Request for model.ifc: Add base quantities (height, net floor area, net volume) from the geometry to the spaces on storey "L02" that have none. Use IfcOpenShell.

First a look at what the model holds.

```python
import ifcopenshell
import ifcopenshell.util.element
import ifcopenshell.util.unit

model = ifcopenshell.open("model.ifc")
print(model.schema)
for unit_type in ("LENGTHUNIT", "AREAUNIT", "VOLUMEUNIT"):
    print(unit_type, ifcopenshell.util.unit.calculate_unit_scale(model, unit_type))
storey = next(s for s in model.by_type("IfcBuildingStorey") if s.Name == "L02")
spaces = [e for e in ifcopenshell.util.element.get_decomposition(storey) if e.is_a("IfcSpace")]
for e in sorted(spaces, key=lambda e: e.id()):
    print(e.id(), e.is_a(), e.Name, list(ifcopenshell.util.element.get_psets(e, qtos_only=True)), sep=" | ")
```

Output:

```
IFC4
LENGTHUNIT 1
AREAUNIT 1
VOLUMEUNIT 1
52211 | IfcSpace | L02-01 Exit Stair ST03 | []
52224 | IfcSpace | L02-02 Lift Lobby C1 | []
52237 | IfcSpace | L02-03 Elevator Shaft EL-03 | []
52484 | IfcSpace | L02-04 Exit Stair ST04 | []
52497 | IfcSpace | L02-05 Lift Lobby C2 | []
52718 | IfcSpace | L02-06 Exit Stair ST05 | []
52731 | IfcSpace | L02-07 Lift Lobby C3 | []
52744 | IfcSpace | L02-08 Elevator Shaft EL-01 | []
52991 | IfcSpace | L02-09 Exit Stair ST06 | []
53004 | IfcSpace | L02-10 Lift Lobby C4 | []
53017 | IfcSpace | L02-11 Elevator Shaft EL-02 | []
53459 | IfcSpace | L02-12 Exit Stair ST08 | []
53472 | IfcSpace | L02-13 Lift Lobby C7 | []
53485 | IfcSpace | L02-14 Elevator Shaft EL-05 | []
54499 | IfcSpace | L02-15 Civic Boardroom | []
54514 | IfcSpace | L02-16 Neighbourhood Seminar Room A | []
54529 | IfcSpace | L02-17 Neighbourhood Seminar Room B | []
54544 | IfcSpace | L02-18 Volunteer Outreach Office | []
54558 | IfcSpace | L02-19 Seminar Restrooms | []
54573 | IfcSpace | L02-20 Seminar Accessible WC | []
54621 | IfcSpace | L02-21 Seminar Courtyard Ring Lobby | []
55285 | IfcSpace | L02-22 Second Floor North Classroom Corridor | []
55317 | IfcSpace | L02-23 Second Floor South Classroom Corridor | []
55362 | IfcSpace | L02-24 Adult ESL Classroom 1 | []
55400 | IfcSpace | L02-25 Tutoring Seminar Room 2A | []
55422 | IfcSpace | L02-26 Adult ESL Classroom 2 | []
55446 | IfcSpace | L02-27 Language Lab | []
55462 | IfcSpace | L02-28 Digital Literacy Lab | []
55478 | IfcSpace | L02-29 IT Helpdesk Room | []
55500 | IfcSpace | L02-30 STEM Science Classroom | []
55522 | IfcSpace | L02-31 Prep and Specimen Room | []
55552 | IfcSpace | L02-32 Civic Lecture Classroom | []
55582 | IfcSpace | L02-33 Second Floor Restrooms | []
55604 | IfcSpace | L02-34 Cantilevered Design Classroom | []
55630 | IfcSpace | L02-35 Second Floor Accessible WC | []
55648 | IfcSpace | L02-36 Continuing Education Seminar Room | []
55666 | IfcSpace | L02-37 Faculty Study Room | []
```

```python
import ifcopenshell
import ifcopenshell.api.pset
import ifcopenshell.geom
import ifcopenshell.util.element
import ifcopenshell.util.shape
import ifcopenshell.util.unit

model = ifcopenshell.open("model.ifc")
unit_scale = ifcopenshell.util.unit.calculate_unit_scale(model)
area_scale = ifcopenshell.util.unit.calculate_unit_scale(model, "AREAUNIT")
volume_scale = ifcopenshell.util.unit.calculate_unit_scale(model, "VOLUMEUNIT")
settings = ifcopenshell.geom.settings()

storey = next(s for s in model.by_type("IfcBuildingStorey") if s.Name == "L02")
spaces = [e for e in ifcopenshell.util.element.get_decomposition(storey) if e.is_a("IfcSpace")]

for e in sorted(spaces, key=lambda e: e.id()):
    if ifcopenshell.util.element.get_psets(e, qtos_only=True, should_inherit=False):
        continue
    # Geometry comes back in metres, in the element's own axes.
    shape = ifcopenshell.geom.create_shape(settings, e)
    values = {
        "Height": ifcopenshell.util.shape.get_z(shape.geometry) / unit_scale,
        "NetFloorArea": ifcopenshell.util.shape.get_footprint_area(shape.geometry) / area_scale,
        "NetVolume": ifcopenshell.util.shape.get_volume(shape.geometry) / volume_scale,
    }
    qto = ifcopenshell.api.pset.add_qto(model, product=e, name="Qto_SpaceBaseQuantities")
    ifcopenshell.api.pset.edit_qto(model, qto=qto, properties=values)
    print(e.id(), {k: round(v, 3) for k, v in values.items()})

model.write("model_v2.ifc")
```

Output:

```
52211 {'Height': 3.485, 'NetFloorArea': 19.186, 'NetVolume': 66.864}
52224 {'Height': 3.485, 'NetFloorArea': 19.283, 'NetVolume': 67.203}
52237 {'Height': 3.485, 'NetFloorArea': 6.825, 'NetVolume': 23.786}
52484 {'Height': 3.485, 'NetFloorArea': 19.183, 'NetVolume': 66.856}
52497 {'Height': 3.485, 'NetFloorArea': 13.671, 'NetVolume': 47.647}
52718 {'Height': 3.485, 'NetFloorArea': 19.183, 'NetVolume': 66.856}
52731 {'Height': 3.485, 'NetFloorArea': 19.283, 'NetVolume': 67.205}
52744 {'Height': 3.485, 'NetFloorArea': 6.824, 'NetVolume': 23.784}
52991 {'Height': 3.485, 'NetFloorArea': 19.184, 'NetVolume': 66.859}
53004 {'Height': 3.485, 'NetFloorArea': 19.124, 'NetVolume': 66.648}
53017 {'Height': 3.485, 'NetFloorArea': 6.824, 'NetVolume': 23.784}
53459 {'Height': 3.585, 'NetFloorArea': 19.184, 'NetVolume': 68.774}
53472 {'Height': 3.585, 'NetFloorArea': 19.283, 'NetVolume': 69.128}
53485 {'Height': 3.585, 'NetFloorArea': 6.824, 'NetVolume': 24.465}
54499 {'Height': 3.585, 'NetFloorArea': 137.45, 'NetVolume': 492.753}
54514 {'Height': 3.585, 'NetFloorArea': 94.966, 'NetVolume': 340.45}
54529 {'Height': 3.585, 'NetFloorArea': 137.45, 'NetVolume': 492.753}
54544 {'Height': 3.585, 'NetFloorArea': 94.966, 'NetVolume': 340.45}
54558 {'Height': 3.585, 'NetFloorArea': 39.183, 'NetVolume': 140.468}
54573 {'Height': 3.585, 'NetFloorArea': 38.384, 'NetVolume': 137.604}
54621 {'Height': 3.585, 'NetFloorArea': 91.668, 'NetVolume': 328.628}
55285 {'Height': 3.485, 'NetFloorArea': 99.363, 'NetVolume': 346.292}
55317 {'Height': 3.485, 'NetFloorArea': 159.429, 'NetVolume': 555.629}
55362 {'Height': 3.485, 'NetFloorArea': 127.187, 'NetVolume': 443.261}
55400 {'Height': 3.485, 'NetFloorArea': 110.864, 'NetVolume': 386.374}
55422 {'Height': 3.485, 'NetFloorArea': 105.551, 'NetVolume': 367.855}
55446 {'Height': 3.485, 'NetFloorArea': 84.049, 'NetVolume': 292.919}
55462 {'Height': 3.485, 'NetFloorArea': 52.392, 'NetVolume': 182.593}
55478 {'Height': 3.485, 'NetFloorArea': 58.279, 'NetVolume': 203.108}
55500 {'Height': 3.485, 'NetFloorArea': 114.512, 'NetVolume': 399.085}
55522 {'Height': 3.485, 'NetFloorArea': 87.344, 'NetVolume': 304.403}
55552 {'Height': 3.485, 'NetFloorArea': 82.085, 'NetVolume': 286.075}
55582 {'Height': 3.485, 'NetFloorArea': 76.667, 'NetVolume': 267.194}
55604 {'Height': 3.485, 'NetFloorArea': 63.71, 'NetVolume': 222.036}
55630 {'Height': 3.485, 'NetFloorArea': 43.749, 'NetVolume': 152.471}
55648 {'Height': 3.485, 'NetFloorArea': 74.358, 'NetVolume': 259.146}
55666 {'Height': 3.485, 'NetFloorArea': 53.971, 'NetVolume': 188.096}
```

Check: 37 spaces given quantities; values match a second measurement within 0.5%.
